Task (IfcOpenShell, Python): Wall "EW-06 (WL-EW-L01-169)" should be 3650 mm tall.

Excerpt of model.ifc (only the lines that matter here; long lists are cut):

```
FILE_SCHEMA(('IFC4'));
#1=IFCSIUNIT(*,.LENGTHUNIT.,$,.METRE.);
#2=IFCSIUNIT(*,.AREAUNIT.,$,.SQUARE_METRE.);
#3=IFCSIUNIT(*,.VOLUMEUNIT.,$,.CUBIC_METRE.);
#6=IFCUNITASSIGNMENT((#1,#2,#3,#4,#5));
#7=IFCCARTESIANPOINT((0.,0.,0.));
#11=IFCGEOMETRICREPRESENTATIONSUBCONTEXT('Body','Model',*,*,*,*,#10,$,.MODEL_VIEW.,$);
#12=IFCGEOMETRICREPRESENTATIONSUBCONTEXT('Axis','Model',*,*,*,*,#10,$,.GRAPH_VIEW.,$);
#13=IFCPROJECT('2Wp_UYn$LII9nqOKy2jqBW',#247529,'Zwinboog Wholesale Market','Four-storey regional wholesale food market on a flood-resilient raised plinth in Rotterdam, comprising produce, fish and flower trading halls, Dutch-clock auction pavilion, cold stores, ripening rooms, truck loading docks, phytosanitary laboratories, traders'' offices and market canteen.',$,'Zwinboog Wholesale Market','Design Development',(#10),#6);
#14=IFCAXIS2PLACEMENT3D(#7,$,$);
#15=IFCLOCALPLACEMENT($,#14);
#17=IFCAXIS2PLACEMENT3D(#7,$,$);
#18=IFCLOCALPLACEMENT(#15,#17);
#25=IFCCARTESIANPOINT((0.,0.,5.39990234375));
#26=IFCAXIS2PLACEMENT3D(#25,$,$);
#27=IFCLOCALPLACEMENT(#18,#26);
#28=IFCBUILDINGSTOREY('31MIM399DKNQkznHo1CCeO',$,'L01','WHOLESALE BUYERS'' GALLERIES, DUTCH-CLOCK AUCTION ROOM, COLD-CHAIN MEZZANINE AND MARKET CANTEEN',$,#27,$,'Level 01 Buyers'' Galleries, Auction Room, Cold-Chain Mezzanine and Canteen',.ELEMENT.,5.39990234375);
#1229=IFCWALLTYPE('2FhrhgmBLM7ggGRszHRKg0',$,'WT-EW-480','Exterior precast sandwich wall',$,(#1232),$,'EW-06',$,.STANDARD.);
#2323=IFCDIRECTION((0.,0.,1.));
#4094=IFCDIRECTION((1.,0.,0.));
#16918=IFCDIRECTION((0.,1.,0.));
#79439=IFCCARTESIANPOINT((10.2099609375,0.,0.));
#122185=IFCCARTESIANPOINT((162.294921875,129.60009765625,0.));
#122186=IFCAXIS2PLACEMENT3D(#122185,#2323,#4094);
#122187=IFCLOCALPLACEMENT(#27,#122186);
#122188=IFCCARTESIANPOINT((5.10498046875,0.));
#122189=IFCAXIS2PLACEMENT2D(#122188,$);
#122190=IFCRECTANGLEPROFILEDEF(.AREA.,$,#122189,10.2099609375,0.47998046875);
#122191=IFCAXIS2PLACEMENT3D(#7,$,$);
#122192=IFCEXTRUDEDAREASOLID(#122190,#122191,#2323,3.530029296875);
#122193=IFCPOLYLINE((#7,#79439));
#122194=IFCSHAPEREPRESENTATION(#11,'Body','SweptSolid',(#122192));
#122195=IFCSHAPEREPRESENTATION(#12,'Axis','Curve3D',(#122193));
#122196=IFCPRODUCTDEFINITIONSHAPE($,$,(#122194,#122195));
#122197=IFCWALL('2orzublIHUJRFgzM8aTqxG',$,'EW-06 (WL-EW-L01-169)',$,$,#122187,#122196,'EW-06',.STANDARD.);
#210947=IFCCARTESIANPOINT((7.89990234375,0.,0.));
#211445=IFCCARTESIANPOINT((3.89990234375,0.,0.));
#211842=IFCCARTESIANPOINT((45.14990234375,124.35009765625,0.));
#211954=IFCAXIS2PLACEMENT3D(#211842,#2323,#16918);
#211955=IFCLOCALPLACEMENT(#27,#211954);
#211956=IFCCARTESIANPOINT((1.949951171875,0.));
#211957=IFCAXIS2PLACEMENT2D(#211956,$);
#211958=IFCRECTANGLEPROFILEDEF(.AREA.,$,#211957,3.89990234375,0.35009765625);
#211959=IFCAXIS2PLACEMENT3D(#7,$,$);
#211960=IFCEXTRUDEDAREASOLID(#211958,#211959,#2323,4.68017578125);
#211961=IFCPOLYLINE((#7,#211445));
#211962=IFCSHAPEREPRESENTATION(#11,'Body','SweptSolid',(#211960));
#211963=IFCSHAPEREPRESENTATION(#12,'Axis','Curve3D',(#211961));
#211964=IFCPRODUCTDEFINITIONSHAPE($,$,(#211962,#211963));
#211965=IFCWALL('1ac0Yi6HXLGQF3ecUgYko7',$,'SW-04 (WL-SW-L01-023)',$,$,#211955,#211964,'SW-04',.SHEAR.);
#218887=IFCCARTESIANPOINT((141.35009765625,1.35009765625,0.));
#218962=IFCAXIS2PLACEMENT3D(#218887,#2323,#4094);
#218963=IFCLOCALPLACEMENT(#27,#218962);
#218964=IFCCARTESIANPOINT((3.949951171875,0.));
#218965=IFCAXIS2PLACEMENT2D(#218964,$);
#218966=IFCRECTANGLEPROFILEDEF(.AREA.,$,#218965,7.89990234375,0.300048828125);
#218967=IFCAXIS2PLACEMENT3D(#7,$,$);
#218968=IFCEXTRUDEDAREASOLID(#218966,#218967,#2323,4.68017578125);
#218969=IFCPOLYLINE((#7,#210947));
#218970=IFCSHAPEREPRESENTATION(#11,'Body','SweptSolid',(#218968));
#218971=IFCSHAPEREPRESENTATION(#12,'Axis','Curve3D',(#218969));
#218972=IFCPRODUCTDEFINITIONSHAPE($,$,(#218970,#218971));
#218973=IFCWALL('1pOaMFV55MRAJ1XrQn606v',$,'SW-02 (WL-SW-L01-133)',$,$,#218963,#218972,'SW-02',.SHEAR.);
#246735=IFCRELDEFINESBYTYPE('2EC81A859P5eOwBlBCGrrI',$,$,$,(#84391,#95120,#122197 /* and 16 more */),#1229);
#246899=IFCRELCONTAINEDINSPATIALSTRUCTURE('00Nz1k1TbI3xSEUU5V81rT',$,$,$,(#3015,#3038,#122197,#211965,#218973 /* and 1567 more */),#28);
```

```python
import ifcopenshell
import ifcopenshell.geom
import ifcopenshell.util.representation
import ifcopenshell.util.shape
import ifcopenshell.util.unit

model = ifcopenshell.open("model.ifc")
unit_scale = ifcopenshell.util.unit.calculate_unit_scale(model)
settings = ifcopenshell.geom.settings()


def volume(element):
    """Net volume in cubic metres, openings subtracted."""
    shape = ifcopenshell.geom.create_shape(settings, element)
    return ifcopenshell.util.shape.get_volume(shape.geometry)


wall = model.by_id(122197)
before = volume(wall)

body = ifcopenshell.util.representation.get_representation(wall, "Model", "Body")
solid = body.Items[0]
old_height = solid.Depth
solid.Depth = 3.65 / unit_scale
after = volume(wall)

print(f"height {old_height:g} -> {solid.Depth:g}, volume {before:.3f} -> {after:.3f} m3")

model.write("model_rev.ifc")
```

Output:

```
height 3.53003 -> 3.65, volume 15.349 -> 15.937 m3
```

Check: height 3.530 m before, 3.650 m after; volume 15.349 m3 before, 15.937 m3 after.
